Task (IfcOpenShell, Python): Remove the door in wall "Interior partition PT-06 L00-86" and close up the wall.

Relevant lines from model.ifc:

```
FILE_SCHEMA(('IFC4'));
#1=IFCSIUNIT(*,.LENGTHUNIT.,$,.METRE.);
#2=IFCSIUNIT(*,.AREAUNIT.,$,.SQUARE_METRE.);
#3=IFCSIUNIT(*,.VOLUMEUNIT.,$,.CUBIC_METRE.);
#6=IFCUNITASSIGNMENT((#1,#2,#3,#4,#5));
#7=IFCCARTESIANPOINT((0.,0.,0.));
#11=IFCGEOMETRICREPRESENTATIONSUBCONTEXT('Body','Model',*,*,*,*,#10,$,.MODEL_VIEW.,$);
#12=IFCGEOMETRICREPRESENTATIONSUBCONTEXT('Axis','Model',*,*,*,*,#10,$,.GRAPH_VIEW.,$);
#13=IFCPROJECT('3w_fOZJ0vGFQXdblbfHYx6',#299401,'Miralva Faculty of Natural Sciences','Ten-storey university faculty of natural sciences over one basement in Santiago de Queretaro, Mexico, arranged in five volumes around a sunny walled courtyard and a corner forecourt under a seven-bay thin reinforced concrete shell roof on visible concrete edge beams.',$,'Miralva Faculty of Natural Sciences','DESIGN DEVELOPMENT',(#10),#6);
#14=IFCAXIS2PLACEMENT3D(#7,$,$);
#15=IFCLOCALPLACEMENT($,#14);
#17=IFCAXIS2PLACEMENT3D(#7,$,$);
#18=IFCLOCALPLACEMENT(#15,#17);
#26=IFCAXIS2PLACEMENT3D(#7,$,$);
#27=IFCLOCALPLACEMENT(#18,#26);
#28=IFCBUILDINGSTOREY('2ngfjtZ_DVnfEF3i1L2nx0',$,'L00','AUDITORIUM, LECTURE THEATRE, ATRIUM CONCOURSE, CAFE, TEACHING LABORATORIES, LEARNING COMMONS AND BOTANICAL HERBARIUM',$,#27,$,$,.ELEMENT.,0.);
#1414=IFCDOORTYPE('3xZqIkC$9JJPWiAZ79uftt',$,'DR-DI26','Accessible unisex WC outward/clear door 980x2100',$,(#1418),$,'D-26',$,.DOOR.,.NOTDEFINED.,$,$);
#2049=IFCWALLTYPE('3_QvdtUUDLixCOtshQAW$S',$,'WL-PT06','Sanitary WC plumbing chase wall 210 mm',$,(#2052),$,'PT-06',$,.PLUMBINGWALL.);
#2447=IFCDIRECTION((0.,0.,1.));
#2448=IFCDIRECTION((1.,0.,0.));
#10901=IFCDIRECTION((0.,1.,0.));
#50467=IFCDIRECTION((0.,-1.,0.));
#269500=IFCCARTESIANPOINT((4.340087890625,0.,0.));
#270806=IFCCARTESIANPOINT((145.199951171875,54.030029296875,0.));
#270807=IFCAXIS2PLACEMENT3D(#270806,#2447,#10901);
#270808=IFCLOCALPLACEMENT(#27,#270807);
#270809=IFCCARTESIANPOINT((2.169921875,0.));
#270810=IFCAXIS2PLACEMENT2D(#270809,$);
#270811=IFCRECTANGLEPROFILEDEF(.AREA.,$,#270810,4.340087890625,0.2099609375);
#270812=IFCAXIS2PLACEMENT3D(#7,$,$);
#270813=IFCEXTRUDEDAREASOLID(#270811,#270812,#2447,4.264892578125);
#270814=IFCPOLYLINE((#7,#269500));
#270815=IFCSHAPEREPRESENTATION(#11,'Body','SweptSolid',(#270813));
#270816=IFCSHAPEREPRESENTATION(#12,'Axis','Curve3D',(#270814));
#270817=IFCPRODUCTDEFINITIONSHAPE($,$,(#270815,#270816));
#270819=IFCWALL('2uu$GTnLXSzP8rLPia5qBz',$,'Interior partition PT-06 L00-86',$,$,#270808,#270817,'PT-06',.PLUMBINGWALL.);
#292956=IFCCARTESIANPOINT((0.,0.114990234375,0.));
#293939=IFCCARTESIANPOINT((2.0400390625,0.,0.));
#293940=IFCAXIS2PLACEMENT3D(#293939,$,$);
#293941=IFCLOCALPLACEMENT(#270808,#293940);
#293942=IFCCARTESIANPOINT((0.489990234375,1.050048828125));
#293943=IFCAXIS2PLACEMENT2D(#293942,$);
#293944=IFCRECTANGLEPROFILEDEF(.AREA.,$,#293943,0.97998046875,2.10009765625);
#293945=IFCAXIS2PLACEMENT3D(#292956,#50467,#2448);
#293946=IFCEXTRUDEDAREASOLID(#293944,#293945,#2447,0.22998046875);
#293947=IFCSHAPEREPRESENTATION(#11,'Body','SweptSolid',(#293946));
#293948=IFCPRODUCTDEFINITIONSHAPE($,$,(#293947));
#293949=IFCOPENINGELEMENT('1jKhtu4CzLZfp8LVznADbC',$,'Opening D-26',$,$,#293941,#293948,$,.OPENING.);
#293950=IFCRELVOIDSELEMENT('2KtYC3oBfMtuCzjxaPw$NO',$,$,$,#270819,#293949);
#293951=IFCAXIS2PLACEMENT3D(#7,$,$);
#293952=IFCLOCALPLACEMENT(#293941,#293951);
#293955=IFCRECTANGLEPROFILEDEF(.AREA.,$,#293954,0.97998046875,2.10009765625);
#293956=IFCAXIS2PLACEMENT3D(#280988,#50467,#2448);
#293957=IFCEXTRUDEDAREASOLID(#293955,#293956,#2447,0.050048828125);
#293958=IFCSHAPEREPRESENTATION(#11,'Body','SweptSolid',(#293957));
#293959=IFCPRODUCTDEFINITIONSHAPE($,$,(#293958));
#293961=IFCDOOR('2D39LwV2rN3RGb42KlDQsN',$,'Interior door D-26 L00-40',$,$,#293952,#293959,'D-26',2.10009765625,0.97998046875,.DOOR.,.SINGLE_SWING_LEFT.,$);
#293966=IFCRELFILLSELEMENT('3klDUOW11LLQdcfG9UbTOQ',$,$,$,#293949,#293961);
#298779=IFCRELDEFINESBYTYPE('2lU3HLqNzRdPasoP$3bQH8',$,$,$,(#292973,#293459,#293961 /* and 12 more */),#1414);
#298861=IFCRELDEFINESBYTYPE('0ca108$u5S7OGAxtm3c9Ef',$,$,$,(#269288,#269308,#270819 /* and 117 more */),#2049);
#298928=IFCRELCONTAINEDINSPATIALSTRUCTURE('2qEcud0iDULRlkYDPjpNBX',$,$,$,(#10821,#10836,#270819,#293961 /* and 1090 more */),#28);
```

```python
import ifcopenshell
import ifcopenshell.api.feature
import ifcopenshell.api.root
import ifcopenshell.geom
import ifcopenshell.util.shape

model = ifcopenshell.open("model.ifc")
settings = ifcopenshell.geom.settings()


def volume(element):
    """Net volume in cubic metres, openings subtracted."""
    shape = ifcopenshell.geom.create_shape(settings, element)
    return ifcopenshell.util.shape.get_volume(shape.geometry)


door = model.by_id(293961)
opening = door.FillsVoids[0].RelatingOpeningElement
wall = opening.VoidsElements[0].RelatingBuildingElement
before = volume(wall)

ifcopenshell.api.root.remove_product(model, product=door)
ifcopenshell.api.feature.remove_feature(model, feature=opening)

after = volume(wall)

print(f"wall volume {before:.3f} -> {after:.3f} m3")

model.write("model_edited.ifc")
```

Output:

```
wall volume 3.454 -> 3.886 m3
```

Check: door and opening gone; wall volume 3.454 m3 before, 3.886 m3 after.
